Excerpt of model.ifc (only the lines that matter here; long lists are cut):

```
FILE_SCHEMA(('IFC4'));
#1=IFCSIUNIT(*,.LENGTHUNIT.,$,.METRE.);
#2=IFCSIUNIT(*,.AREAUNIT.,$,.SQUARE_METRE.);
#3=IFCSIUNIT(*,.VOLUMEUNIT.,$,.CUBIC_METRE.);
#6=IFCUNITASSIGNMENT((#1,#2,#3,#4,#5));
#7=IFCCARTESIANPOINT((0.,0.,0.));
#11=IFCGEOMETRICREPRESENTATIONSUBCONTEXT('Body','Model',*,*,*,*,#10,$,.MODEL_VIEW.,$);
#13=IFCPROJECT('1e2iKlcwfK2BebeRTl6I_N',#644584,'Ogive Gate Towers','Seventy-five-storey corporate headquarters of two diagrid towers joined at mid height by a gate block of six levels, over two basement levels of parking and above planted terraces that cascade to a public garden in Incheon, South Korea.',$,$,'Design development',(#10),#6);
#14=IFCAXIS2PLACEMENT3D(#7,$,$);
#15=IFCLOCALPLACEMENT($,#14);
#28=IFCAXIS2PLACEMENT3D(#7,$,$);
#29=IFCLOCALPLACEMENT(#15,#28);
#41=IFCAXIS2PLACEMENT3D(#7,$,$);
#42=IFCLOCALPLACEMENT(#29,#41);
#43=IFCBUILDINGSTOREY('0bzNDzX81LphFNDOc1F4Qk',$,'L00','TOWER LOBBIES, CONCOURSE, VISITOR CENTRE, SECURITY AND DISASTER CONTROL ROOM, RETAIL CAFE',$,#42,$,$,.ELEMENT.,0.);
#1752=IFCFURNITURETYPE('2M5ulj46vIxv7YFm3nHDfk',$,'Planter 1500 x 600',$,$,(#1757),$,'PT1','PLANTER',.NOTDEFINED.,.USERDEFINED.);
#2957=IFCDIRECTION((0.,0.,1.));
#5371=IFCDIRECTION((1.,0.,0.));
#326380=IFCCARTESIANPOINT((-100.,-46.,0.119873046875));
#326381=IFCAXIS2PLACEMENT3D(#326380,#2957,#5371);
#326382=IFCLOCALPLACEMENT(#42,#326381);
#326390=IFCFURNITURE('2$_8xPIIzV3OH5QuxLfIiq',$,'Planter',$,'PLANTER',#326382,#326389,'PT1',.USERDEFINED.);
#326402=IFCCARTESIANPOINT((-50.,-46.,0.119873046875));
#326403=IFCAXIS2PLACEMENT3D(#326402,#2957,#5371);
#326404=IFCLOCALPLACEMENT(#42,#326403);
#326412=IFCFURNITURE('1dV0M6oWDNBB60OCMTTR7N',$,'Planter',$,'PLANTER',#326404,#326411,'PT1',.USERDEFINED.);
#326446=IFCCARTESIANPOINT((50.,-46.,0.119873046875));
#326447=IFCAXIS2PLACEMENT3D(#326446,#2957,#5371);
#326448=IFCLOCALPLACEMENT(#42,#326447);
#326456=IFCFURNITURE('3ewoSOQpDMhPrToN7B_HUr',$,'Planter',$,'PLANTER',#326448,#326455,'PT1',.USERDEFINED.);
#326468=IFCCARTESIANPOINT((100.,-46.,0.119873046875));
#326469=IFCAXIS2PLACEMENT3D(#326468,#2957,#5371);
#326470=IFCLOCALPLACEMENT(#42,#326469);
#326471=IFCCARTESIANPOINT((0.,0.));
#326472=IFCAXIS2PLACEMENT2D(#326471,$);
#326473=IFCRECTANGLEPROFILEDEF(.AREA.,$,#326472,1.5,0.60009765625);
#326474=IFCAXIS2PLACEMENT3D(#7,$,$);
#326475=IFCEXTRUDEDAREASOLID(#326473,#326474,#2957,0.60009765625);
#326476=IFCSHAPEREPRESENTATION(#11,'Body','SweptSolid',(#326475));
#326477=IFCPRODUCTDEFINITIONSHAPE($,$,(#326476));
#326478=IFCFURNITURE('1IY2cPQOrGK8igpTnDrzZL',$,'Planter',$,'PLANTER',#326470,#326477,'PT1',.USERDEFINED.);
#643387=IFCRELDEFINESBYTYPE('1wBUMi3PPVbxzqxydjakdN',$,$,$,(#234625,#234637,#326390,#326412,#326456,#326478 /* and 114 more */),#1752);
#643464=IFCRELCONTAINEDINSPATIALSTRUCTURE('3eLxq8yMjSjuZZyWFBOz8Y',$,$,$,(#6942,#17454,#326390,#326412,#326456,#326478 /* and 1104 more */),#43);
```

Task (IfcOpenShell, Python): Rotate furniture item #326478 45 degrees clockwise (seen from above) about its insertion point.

```python
import ifcopenshell
import ifcopenshell.api.geometry
import ifcopenshell.util.placement

model = ifcopenshell.open("model.ifc")

item = model.by_id(326478)
matrix = ifcopenshell.util.placement.get_local_placement(item.ObjectPlacement)
matrix = matrix @ ifcopenshell.util.placement.rotation(-45, "Z")
ifcopenshell.api.geometry.edit_object_placement(model, product=item, matrix=matrix, is_si=False)

print(ifcopenshell.util.placement.get_local_placement(item.ObjectPlacement).round(3) + 0.0)

model.write("model_rev.ifc")
```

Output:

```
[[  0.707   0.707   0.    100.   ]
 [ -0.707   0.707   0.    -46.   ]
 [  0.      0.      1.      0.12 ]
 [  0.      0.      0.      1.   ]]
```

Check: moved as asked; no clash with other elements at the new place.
